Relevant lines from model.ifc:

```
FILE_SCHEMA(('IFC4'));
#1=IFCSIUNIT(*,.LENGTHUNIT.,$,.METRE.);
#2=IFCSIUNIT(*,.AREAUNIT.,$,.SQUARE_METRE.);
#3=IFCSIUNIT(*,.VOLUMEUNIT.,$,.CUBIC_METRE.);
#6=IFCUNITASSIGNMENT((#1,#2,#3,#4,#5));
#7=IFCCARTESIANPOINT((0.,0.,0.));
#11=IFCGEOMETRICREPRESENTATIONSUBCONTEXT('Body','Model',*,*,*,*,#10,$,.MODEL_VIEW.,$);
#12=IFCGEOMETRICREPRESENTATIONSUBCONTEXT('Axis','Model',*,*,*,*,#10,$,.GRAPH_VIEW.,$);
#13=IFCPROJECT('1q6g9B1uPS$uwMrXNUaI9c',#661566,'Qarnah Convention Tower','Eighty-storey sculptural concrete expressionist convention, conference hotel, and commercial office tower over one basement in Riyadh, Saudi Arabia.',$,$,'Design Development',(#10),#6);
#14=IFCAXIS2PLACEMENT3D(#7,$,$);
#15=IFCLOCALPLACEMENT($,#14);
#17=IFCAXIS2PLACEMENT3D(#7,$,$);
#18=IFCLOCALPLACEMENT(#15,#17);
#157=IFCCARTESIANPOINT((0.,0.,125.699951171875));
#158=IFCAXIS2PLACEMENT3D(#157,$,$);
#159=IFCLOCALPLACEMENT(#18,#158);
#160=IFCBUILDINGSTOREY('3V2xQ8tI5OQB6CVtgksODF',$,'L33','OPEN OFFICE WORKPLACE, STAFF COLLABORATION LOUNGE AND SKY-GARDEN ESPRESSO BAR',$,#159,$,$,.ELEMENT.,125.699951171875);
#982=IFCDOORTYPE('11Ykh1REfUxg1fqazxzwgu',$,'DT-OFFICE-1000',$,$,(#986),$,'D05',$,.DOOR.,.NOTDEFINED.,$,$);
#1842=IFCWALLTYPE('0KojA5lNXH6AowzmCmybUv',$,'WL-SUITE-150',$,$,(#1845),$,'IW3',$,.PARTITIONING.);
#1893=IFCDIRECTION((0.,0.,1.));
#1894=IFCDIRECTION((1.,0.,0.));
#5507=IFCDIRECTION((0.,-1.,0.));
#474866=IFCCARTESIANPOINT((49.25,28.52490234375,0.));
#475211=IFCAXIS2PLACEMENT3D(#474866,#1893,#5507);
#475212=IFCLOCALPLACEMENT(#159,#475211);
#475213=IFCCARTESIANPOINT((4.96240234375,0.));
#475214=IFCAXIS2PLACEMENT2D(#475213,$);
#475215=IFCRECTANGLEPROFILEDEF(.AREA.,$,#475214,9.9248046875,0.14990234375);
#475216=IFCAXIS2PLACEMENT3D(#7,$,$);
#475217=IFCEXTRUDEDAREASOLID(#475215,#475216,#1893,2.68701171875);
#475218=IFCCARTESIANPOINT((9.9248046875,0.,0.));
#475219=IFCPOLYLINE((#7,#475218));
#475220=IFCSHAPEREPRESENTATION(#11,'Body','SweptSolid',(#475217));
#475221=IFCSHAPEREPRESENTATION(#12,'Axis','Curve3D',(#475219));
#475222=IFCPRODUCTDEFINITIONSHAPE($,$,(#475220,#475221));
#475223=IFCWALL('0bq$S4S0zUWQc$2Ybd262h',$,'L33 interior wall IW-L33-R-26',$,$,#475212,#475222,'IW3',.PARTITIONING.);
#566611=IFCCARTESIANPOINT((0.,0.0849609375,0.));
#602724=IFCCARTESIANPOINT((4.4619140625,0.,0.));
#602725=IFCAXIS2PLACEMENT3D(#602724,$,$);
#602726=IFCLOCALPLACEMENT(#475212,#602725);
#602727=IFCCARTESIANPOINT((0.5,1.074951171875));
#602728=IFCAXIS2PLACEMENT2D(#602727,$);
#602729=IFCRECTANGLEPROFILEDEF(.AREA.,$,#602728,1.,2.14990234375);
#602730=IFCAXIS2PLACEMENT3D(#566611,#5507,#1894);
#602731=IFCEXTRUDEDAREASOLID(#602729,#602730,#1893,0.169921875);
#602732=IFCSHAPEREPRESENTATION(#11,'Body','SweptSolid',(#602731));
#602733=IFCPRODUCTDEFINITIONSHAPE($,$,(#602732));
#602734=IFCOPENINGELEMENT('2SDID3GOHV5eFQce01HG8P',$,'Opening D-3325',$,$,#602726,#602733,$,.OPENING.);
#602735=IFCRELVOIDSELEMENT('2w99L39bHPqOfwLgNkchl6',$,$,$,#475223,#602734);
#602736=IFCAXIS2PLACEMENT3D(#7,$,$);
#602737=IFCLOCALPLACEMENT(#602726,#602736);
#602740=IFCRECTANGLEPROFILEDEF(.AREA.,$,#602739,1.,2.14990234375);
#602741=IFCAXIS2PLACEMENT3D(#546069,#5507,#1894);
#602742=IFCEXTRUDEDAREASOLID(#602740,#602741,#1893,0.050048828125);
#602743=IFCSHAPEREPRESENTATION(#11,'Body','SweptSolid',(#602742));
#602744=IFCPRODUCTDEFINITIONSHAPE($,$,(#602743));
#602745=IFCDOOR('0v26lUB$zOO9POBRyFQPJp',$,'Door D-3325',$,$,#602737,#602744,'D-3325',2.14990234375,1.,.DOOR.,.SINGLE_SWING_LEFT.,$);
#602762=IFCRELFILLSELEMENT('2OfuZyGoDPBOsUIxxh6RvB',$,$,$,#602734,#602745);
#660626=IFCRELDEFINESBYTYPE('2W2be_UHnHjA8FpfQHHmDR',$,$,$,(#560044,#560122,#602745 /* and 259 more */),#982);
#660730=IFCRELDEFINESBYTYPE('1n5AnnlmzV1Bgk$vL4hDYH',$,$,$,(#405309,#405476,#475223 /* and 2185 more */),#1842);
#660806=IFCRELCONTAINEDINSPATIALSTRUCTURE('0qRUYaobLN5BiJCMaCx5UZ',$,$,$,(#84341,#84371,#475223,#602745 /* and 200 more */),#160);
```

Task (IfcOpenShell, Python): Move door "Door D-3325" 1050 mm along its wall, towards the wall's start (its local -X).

```python
import ifcopenshell
import ifcopenshell.api.geometry
import ifcopenshell.util.placement

model = ifcopenshell.open("model.ifc")

door = model.by_id(602745)
opening = door.FillsVoids[0].RelatingOpeningElement
wall = opening.VoidsElements[0].RelatingBuildingElement

wall_matrix = ifcopenshell.util.placement.get_local_placement(wall.ObjectPlacement)
shift = wall_matrix[:3, 0] * -1.05
before = ifcopenshell.util.placement.get_local_placement(door.ObjectPlacement)[:3, 3].copy()

# The door is placed relative to its opening, so it follows when the opening moves.
matrix = ifcopenshell.util.placement.get_local_placement(opening.ObjectPlacement)
matrix[:3, 3] += shift
ifcopenshell.api.geometry.edit_object_placement(
    model, product=opening, matrix=matrix, is_si=False, should_transform_children=True
)

after = ifcopenshell.util.placement.get_local_placement(door.ObjectPlacement)[:3, 3]
print("door moved by", (after - before).round(3) + 0.0)

model.write("model_v2.ifc")
```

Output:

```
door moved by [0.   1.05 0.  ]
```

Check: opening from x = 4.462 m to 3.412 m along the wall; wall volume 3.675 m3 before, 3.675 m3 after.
